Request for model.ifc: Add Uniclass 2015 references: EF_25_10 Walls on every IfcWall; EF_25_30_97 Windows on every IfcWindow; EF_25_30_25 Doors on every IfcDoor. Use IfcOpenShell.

First a look at what the model holds.

```python
import ifcopenshell

model = ifcopenshell.open("model.ifc")
print(model.schema)
print("classifications:", [c.Name for c in model.by_type("IfcClassification")])
for ifc_class in ("IfcDoor", "IfcRoof", "IfcStair", "IfcWall", "IfcWindow"):
    print(ifc_class, len(model.by_type(ifc_class)))
```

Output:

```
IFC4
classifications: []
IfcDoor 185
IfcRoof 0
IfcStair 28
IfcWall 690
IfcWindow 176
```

```python
import ifcopenshell
import ifcopenshell.api.classification

model = ifcopenshell.open("model.ifc")

system = ifcopenshell.api.classification.add_classification(model, classification="Uniclass 2015")

codes = {
    "IfcWall": ("EF_25_10", "Walls"),
    "IfcWindow": ("EF_25_30_97", "Windows"),
    "IfcDoor": ("EF_25_30_25", "Doors"),
}
for ifc_class, (code, name) in codes.items():
    products = model.by_type(ifc_class)
    ifcopenshell.api.classification.add_reference(
        model, products=products, classification=system, identification=code, name=name
    )
    print(code, len(products))

model.write("model-out.ifc")
```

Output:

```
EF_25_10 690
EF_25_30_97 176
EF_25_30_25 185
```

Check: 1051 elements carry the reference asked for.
